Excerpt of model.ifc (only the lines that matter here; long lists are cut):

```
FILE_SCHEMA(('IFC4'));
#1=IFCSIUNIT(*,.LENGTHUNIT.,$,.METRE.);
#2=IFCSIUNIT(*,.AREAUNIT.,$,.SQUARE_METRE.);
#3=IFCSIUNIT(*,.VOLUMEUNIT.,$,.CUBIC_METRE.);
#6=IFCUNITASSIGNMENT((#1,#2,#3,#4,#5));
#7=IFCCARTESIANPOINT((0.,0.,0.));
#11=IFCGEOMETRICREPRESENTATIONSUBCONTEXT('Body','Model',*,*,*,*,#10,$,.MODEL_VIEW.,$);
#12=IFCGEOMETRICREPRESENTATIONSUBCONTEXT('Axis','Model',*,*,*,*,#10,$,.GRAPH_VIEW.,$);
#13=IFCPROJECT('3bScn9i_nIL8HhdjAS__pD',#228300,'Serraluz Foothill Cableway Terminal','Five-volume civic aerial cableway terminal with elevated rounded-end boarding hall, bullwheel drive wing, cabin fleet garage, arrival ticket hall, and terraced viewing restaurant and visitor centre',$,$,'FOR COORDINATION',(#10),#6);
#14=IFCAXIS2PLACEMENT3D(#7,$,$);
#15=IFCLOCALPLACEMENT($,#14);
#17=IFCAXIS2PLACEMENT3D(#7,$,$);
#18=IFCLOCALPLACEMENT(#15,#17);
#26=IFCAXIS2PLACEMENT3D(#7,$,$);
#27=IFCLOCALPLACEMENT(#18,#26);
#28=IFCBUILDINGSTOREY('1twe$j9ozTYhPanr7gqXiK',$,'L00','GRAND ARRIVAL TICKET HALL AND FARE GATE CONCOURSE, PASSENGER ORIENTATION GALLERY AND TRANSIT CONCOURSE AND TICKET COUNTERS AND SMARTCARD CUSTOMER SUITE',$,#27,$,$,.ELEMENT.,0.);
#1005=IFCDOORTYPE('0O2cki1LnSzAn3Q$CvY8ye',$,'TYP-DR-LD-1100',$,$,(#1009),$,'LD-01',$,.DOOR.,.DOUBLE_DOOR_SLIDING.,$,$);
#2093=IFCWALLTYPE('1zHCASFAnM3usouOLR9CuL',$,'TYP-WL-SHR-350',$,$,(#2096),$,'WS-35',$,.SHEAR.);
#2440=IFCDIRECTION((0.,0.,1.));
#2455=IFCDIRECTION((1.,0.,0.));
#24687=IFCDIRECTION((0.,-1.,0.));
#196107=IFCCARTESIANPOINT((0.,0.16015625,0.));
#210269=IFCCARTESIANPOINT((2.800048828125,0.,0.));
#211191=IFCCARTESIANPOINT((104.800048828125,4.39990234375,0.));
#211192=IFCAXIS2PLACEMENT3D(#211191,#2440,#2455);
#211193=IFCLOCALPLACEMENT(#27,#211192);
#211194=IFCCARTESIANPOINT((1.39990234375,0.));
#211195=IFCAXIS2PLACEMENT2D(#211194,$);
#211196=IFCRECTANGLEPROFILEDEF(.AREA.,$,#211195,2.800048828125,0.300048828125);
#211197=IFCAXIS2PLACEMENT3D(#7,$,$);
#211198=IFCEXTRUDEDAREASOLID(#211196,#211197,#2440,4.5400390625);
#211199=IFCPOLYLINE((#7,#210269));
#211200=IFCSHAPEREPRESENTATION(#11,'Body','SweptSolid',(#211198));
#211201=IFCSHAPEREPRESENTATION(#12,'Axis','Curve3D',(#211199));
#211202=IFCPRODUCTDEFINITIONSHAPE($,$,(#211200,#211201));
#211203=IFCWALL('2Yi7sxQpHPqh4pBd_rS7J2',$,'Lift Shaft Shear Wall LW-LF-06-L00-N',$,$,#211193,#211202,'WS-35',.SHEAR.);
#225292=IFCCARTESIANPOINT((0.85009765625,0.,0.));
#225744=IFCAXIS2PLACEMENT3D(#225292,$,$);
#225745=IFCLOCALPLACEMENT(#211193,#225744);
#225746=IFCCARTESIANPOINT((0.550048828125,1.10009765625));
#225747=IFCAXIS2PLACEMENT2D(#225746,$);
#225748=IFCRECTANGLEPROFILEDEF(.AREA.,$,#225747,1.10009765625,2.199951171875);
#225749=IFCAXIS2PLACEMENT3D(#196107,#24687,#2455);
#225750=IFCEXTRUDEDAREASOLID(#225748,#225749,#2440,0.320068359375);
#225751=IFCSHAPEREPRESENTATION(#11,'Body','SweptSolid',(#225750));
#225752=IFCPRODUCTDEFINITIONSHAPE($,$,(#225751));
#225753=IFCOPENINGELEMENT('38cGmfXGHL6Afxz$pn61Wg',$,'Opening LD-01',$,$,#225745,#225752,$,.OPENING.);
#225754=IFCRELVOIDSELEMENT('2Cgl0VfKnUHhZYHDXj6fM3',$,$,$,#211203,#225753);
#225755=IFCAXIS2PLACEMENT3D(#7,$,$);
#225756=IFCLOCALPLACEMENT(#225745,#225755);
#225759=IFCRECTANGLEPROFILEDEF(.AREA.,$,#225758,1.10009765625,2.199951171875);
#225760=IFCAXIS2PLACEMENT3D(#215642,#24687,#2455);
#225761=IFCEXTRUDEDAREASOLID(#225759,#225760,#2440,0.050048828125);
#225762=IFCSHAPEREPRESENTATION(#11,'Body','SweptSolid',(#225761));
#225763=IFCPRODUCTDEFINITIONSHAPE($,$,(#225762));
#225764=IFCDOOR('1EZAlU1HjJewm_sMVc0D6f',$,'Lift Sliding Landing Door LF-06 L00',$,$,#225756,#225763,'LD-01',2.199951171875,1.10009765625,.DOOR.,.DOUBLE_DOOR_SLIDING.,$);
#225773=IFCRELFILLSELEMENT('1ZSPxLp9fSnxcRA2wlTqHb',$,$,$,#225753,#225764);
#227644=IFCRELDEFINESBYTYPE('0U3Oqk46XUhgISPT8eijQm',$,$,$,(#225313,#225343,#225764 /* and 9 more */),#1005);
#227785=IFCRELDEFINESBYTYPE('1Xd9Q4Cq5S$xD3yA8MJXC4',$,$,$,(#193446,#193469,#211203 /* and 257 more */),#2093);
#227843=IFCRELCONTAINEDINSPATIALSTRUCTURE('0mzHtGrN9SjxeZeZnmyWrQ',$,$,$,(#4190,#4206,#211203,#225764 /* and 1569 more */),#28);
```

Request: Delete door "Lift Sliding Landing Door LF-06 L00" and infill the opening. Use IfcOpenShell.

```python
import ifcopenshell
import ifcopenshell.api.feature
import ifcopenshell.api.root
import ifcopenshell.geom
import ifcopenshell.util.shape

model = ifcopenshell.open("model.ifc")
settings = ifcopenshell.geom.settings()


def volume(element):
    """Net volume in cubic metres, openings subtracted."""
    shape = ifcopenshell.geom.create_shape(settings, element)
    return ifcopenshell.util.shape.get_volume(shape.geometry)


door = model.by_guid("1EZAlU1HjJewm_sMVc0D6f")
opening = door.FillsVoids[0].RelatingOpeningElement
wall = opening.VoidsElements[0].RelatingBuildingElement
before = volume(wall)

ifcopenshell.api.root.remove_product(model, product=door)
ifcopenshell.api.feature.remove_feature(model, feature=opening)

after = volume(wall)

print(f"wall volume {before:.3f} -> {after:.3f} m3")

model.write("model_rev.ifc")
```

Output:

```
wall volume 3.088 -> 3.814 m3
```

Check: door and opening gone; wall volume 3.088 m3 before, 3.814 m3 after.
